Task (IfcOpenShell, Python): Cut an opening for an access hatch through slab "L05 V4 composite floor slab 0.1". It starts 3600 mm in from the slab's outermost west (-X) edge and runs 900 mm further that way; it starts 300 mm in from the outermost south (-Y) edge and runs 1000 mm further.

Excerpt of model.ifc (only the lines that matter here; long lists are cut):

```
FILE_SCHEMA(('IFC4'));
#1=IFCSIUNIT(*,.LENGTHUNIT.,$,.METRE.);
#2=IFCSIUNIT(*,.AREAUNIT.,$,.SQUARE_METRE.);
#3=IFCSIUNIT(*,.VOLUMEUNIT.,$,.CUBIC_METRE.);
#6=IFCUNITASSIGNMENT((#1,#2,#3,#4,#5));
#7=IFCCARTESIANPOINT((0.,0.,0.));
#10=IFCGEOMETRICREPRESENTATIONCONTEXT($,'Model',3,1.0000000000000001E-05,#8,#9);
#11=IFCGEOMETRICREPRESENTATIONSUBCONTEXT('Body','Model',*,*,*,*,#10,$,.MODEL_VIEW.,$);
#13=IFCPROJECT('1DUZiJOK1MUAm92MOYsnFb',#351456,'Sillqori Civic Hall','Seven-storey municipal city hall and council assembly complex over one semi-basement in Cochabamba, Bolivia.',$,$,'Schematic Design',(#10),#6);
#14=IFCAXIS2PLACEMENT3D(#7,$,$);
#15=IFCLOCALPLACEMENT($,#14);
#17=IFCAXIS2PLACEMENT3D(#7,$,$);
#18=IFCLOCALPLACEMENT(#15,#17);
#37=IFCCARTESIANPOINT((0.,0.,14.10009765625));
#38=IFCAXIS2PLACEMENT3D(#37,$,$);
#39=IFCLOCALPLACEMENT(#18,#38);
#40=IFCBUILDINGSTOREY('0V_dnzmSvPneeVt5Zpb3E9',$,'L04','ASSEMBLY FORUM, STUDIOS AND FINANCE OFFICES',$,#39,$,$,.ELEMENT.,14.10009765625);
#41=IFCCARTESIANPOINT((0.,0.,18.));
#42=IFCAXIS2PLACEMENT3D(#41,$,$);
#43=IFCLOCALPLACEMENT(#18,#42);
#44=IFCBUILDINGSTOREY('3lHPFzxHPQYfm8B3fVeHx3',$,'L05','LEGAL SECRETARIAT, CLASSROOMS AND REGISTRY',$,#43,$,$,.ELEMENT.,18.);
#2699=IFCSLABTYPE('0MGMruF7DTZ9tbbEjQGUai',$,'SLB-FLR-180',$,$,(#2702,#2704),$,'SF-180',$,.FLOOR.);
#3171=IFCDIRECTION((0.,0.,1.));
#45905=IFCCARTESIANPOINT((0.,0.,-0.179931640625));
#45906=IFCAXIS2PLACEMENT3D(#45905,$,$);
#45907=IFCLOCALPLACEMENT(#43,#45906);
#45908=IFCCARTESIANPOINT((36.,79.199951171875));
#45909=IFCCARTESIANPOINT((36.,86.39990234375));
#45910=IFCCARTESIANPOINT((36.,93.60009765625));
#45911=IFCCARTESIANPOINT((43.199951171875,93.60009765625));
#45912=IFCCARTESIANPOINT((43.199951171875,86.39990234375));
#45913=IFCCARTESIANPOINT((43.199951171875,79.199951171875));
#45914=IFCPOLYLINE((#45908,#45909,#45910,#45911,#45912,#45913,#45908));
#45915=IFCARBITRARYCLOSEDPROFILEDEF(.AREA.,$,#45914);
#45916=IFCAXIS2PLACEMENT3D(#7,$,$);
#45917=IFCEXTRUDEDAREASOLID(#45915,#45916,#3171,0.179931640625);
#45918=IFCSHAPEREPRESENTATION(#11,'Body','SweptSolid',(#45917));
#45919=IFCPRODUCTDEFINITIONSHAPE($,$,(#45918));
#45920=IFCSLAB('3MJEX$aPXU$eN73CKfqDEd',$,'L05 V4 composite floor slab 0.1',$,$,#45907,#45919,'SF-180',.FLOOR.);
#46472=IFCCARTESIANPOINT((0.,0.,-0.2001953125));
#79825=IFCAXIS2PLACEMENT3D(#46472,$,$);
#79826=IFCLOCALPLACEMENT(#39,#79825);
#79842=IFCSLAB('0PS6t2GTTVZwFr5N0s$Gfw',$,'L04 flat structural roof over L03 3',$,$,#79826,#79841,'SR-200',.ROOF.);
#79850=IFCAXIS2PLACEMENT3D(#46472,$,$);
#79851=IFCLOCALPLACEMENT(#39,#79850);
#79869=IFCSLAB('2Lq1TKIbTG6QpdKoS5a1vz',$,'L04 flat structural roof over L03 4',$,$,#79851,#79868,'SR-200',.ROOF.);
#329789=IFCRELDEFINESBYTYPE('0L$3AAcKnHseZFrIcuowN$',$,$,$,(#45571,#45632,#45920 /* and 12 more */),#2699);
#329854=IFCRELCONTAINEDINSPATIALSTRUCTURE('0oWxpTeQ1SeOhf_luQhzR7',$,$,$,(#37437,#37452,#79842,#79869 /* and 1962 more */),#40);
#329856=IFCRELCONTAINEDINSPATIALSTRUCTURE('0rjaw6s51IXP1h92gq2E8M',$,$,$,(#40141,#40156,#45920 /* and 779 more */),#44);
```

```python
import numpy as np
import ifcopenshell
import ifcopenshell.api.feature
import ifcopenshell.api.geometry
import ifcopenshell.api.root
import ifcopenshell.geom
import ifcopenshell.util.placement
import ifcopenshell.util.representation
import ifcopenshell.util.shape
import ifcopenshell.util.unit

model = ifcopenshell.open("model.ifc")
unit_scale = ifcopenshell.util.unit.calculate_unit_scale(model)
settings = ifcopenshell.geom.settings()


def volume(element):
    """Net volume in cubic metres, openings subtracted."""
    shape = ifcopenshell.geom.create_shape(settings, element)
    return ifcopenshell.util.shape.get_volume(shape.geometry)


slab = model.by_id(45920)
before = volume(slab)

# Extent in the slab's own axes, in metres. The edges named are its -X and -Y sides.
slab_shape = ifcopenshell.geom.create_shape(settings, slab)
vertices = ifcopenshell.util.shape.get_vertices(slab_shape.geometry)
x_min, y_min, bottom = vertices.min(axis=0)
top = vertices[:, 2].max()

opening = ifcopenshell.api.root.create_entity(model, ifc_class="IfcOpeningElement", name="Access hatch opening", predefined_type="OPENING")
context = ifcopenshell.util.representation.get_context(model, "Model", "Body", "MODEL_VIEW")
width, depth = 0.9, 1
outline = [(0.0, 0.0), (width, 0.0), (width, depth), (0.0, depth), (0.0, 0.0)]
# Overshoot both faces by 50 mm so the cut is clean.
shape = ifcopenshell.api.geometry.add_slab_representation(
    model, context=context, depth=top - bottom + 0.1, polyline=outline
)
ifcopenshell.api.geometry.assign_representation(model, product=opening, representation=shape)

matrix = ifcopenshell.util.placement.get_local_placement(slab.ObjectPlacement)
matrix[:, 3] = matrix @ np.append(np.array([x_min + 3.6, y_min + 0.3, bottom - 0.05]) / unit_scale, 1.0)
ifcopenshell.api.geometry.edit_object_placement(model, product=opening, matrix=matrix, is_si=False)
ifcopenshell.api.feature.add_feature(model, feature=opening, element=slab)

after = volume(slab)

print(f"slab volume {before:.3f} -> {after:.3f} m3")

model.write("model_rev.ifc")
```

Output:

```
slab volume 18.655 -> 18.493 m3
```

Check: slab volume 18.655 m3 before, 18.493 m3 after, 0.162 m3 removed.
